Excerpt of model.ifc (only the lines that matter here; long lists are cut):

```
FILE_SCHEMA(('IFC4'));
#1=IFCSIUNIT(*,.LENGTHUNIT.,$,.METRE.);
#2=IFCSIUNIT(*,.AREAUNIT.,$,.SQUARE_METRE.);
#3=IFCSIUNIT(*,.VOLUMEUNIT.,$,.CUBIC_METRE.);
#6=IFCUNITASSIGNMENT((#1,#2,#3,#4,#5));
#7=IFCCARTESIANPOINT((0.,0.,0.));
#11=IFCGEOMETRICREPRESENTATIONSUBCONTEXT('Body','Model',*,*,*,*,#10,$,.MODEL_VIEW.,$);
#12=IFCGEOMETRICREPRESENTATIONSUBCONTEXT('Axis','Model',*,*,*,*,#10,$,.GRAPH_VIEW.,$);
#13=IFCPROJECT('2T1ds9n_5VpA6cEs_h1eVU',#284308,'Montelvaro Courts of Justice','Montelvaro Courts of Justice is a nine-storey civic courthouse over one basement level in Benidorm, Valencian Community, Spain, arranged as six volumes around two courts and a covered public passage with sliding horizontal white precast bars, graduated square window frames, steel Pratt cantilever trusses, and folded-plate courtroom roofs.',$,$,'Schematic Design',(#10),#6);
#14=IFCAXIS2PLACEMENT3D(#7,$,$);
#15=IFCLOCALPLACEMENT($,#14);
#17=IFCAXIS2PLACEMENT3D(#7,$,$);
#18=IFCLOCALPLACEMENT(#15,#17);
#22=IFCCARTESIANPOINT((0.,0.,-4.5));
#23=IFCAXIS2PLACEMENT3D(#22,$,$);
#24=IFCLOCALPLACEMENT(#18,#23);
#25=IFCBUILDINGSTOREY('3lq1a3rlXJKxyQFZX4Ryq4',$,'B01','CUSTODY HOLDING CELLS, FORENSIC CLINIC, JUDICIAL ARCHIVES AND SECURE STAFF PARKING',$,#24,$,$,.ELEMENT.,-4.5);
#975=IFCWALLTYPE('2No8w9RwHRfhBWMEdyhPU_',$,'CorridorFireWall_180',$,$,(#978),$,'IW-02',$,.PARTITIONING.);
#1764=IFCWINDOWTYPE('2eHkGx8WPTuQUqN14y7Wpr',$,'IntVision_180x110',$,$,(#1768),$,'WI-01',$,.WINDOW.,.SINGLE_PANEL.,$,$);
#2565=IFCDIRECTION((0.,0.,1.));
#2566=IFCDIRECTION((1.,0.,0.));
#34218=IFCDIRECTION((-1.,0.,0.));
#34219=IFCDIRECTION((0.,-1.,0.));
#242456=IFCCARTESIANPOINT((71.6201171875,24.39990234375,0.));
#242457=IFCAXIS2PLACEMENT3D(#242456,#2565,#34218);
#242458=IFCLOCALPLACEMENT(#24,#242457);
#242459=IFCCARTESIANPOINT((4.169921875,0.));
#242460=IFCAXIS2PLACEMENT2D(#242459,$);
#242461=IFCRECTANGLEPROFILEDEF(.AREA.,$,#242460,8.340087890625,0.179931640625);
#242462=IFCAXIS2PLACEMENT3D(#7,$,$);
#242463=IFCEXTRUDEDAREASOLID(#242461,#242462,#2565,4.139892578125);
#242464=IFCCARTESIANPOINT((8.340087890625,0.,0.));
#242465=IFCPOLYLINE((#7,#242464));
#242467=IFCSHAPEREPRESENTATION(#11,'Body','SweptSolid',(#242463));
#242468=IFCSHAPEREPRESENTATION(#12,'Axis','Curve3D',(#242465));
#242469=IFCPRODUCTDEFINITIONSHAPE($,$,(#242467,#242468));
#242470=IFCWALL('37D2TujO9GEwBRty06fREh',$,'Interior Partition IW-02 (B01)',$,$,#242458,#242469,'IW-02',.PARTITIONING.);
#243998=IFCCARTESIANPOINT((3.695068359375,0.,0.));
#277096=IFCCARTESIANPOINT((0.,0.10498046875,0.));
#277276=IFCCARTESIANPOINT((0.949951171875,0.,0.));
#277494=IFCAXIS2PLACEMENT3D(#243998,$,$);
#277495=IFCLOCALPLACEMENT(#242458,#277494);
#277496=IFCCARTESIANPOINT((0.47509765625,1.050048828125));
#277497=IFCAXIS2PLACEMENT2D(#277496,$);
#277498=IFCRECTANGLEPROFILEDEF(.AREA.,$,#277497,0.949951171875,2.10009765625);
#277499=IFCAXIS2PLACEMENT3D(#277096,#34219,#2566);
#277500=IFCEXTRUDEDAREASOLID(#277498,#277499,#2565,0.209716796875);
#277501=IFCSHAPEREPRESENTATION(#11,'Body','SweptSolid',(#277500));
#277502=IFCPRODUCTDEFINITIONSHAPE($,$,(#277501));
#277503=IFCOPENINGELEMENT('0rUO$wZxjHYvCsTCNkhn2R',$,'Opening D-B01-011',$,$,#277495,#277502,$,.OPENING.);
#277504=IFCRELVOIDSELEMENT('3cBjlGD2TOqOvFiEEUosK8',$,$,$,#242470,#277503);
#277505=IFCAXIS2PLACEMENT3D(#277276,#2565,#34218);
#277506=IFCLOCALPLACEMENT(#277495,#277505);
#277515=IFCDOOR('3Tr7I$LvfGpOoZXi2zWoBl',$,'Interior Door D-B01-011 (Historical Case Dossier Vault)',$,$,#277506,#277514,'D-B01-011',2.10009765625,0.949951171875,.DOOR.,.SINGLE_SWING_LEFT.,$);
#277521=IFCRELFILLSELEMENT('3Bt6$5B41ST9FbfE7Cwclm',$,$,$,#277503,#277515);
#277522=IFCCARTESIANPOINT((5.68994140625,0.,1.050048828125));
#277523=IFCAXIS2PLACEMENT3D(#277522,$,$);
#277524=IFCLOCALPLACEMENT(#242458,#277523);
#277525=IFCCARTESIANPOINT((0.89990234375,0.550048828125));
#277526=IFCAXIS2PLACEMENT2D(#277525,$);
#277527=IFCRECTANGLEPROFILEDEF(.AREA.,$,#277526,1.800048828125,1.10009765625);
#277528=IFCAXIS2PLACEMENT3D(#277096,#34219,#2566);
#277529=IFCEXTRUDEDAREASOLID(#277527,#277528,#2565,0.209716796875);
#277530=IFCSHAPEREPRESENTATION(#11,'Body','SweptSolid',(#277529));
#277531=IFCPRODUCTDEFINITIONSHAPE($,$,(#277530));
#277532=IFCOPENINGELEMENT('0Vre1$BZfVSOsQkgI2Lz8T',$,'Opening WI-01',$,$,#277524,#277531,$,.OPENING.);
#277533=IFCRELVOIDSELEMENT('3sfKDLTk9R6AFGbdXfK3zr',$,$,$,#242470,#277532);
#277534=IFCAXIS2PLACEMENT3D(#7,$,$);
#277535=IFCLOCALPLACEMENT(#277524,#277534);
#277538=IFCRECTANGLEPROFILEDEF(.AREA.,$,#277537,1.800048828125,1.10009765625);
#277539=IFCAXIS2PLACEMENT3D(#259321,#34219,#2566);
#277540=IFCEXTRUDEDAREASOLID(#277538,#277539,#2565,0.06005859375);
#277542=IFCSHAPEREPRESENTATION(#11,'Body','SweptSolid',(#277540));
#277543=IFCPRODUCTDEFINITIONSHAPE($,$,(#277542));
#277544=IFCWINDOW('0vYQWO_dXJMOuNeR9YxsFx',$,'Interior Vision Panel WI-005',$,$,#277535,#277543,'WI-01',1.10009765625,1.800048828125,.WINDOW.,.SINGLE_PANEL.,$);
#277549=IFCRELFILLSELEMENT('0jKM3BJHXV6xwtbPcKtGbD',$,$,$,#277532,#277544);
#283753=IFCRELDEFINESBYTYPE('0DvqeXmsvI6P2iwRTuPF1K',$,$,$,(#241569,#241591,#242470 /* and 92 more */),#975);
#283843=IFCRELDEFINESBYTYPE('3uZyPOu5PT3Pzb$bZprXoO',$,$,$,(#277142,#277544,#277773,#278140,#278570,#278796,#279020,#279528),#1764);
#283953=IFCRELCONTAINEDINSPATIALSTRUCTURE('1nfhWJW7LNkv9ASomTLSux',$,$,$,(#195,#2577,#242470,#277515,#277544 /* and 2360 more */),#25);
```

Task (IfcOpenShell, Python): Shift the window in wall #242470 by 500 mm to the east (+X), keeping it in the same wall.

```python
import ifcopenshell
import ifcopenshell.api.geometry
import ifcopenshell.util.placement

model = ifcopenshell.open("model.ifc")

window = model.by_guid("0vYQWO_dXJMOuNeR9YxsFx")
opening = window.FillsVoids[0].RelatingOpeningElement
wall = opening.VoidsElements[0].RelatingBuildingElement

wall_matrix = ifcopenshell.util.placement.get_local_placement(wall.ObjectPlacement)
shift = wall_matrix[:3, 0] * -0.5
before = ifcopenshell.util.placement.get_local_placement(window.ObjectPlacement)[:3, 3].copy()

# The window is placed relative to its opening, so it follows when the opening moves.
matrix = ifcopenshell.util.placement.get_local_placement(opening.ObjectPlacement)
matrix[:3, 3] += shift
ifcopenshell.api.geometry.edit_object_placement(
    model, product=opening, matrix=matrix, is_si=False, should_transform_children=True
)

after = ifcopenshell.util.placement.get_local_placement(window.ObjectPlacement)[:3, 3]
print("window moved by", (after - before).round(3) + 0.0)

model.write("model_rev.ifc")
```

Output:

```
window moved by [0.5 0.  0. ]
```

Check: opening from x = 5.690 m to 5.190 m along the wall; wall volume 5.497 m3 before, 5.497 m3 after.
